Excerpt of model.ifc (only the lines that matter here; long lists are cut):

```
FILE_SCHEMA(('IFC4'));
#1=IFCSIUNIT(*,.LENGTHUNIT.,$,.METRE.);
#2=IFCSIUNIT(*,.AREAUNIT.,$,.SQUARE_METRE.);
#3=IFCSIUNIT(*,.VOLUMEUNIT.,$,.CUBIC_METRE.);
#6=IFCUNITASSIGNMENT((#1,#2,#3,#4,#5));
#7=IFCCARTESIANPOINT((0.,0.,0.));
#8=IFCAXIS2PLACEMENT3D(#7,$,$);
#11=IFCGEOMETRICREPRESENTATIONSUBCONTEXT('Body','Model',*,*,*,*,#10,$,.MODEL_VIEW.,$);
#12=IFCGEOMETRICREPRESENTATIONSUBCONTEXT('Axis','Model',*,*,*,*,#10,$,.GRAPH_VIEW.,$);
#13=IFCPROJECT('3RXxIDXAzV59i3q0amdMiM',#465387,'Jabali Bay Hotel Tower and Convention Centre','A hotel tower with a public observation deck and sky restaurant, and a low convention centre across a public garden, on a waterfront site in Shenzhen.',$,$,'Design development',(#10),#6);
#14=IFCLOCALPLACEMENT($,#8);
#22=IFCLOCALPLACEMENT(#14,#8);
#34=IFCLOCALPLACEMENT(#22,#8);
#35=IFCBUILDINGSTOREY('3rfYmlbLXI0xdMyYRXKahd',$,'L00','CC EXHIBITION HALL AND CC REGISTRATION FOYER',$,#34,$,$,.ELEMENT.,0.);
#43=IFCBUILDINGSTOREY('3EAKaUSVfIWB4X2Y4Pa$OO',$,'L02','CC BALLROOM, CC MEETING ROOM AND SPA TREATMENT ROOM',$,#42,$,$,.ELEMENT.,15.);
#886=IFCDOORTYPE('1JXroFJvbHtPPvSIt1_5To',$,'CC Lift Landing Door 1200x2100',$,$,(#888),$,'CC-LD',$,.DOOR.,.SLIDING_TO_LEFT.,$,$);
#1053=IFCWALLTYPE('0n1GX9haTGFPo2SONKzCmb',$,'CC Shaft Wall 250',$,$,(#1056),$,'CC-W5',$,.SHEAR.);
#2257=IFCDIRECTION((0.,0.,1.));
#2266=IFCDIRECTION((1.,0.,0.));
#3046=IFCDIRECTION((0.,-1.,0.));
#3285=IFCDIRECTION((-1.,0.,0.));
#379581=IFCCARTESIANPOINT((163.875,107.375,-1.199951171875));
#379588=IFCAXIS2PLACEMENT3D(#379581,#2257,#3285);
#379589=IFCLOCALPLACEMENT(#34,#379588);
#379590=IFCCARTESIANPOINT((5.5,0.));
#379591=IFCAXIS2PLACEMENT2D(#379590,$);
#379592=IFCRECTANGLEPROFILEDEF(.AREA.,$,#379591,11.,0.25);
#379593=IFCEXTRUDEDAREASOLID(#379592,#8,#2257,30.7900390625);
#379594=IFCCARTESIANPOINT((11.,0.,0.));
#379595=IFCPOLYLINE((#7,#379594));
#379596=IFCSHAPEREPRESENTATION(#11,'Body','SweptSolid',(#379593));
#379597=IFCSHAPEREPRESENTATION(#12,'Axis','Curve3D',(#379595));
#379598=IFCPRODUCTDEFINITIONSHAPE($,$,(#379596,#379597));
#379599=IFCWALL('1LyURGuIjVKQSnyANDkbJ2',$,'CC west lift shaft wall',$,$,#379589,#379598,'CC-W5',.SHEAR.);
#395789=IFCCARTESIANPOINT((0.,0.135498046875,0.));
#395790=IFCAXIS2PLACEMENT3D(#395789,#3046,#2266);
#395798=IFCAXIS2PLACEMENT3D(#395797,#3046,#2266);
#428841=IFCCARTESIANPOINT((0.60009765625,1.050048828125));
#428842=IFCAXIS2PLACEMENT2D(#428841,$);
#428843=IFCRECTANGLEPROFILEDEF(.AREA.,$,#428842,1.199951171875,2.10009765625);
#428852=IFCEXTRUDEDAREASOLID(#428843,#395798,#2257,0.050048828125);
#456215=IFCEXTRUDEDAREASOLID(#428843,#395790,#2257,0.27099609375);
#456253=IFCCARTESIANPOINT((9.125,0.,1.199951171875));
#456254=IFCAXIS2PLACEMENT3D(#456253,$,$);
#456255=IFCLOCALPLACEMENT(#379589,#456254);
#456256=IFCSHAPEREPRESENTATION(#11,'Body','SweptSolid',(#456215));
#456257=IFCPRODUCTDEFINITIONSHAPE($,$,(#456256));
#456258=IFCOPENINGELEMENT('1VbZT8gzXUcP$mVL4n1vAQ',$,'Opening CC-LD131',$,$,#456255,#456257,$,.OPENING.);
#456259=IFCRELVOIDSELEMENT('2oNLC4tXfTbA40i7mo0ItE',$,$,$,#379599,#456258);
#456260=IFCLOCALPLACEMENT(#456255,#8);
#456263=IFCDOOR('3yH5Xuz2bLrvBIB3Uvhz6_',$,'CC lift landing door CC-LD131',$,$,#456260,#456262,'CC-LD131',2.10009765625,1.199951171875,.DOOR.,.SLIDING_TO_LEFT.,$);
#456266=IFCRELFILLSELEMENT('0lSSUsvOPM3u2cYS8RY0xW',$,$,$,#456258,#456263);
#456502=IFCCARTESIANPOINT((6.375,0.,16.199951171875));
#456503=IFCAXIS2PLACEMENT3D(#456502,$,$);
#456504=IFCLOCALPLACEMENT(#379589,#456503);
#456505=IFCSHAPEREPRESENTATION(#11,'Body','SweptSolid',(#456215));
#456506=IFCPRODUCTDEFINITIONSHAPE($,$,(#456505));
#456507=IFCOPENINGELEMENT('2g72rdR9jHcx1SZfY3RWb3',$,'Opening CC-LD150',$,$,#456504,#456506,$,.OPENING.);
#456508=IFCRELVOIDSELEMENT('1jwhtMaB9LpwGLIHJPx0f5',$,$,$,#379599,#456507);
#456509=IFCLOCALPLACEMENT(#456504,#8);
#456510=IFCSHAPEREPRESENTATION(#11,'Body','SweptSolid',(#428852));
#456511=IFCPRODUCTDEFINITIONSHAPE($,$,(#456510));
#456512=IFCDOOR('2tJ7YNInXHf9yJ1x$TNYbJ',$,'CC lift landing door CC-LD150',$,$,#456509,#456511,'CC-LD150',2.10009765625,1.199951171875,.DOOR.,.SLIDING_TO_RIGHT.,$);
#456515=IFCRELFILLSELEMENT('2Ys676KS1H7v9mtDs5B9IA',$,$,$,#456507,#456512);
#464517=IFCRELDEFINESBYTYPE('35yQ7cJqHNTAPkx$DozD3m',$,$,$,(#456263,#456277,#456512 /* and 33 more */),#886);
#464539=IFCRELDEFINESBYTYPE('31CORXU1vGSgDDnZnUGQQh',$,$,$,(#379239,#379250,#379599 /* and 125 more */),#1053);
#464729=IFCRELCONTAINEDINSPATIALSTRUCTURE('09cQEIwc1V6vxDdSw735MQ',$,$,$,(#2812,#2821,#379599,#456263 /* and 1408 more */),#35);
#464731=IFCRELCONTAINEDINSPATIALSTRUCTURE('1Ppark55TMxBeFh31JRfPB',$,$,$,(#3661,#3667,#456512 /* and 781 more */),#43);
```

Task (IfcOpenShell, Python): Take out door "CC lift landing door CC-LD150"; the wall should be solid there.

```python
import ifcopenshell
import ifcopenshell.api.feature
import ifcopenshell.api.root
import ifcopenshell.geom
import ifcopenshell.util.shape

model = ifcopenshell.open("model.ifc")
settings = ifcopenshell.geom.settings()


def volume(element):
    """Net volume in cubic metres, openings subtracted."""
    shape = ifcopenshell.geom.create_shape(settings, element)
    return ifcopenshell.util.shape.get_volume(shape.geometry)


door = model.by_guid("2tJ7YNInXHf9yJ1x$TNYbJ")
opening = door.FillsVoids[0].RelatingOpeningElement
wall = opening.VoidsElements[0].RelatingBuildingElement
before = volume(wall)

ifcopenshell.api.root.remove_product(model, product=door)
ifcopenshell.api.feature.remove_feature(model, feature=opening)

after = volume(wall)

print(f"wall volume {before:.3f} -> {after:.3f} m3")

model.write("model_edited.ifc")
```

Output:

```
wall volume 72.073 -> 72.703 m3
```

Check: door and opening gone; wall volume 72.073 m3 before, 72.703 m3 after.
